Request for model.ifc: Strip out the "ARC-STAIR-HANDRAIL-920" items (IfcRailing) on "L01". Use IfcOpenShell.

First a look at what the model holds.

```python
import ifcopenshell
import ifcopenshell.util.element

model = ifcopenshell.open("model.ifc")
print(model.schema)
storey = next(s for s in model.by_type("IfcBuildingStorey") if s.Name == "L01")
railings = [e for e in ifcopenshell.util.element.get_decomposition(storey) if e.is_a("IfcRailing")]
seen = {}
for e in railings:
    element_type = ifcopenshell.util.element.get_type(e)
    name = element_type.Name if element_type not in (None, e) else None
    seen[name] = seen.get(name, 0) + 1
for name, count in sorted(seen.items(), key=str):
    print(count, "x", name)
```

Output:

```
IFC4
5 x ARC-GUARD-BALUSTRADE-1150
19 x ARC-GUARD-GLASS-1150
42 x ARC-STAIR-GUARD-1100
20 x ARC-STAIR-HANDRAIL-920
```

```python
import ifcopenshell
import ifcopenshell.api.root
import ifcopenshell.util.element

model = ifcopenshell.open("model.ifc")

storey = next(s for s in model.by_type("IfcBuildingStorey") if s.Name == "L01")
railings = [e for e in ifcopenshell.util.element.get_decomposition(storey) if e.is_a("IfcRailing")]
targets = [e for e in railings if (t := ifcopenshell.util.element.get_type(e)) not in (None, e) and t.Name == "ARC-STAIR-HANDRAIL-920"]

for e in targets:
    ifcopenshell.api.root.remove_product(model, product=e)
print(len(targets), "removed")

model.write("model_rev.ifc")
```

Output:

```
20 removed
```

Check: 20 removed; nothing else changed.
